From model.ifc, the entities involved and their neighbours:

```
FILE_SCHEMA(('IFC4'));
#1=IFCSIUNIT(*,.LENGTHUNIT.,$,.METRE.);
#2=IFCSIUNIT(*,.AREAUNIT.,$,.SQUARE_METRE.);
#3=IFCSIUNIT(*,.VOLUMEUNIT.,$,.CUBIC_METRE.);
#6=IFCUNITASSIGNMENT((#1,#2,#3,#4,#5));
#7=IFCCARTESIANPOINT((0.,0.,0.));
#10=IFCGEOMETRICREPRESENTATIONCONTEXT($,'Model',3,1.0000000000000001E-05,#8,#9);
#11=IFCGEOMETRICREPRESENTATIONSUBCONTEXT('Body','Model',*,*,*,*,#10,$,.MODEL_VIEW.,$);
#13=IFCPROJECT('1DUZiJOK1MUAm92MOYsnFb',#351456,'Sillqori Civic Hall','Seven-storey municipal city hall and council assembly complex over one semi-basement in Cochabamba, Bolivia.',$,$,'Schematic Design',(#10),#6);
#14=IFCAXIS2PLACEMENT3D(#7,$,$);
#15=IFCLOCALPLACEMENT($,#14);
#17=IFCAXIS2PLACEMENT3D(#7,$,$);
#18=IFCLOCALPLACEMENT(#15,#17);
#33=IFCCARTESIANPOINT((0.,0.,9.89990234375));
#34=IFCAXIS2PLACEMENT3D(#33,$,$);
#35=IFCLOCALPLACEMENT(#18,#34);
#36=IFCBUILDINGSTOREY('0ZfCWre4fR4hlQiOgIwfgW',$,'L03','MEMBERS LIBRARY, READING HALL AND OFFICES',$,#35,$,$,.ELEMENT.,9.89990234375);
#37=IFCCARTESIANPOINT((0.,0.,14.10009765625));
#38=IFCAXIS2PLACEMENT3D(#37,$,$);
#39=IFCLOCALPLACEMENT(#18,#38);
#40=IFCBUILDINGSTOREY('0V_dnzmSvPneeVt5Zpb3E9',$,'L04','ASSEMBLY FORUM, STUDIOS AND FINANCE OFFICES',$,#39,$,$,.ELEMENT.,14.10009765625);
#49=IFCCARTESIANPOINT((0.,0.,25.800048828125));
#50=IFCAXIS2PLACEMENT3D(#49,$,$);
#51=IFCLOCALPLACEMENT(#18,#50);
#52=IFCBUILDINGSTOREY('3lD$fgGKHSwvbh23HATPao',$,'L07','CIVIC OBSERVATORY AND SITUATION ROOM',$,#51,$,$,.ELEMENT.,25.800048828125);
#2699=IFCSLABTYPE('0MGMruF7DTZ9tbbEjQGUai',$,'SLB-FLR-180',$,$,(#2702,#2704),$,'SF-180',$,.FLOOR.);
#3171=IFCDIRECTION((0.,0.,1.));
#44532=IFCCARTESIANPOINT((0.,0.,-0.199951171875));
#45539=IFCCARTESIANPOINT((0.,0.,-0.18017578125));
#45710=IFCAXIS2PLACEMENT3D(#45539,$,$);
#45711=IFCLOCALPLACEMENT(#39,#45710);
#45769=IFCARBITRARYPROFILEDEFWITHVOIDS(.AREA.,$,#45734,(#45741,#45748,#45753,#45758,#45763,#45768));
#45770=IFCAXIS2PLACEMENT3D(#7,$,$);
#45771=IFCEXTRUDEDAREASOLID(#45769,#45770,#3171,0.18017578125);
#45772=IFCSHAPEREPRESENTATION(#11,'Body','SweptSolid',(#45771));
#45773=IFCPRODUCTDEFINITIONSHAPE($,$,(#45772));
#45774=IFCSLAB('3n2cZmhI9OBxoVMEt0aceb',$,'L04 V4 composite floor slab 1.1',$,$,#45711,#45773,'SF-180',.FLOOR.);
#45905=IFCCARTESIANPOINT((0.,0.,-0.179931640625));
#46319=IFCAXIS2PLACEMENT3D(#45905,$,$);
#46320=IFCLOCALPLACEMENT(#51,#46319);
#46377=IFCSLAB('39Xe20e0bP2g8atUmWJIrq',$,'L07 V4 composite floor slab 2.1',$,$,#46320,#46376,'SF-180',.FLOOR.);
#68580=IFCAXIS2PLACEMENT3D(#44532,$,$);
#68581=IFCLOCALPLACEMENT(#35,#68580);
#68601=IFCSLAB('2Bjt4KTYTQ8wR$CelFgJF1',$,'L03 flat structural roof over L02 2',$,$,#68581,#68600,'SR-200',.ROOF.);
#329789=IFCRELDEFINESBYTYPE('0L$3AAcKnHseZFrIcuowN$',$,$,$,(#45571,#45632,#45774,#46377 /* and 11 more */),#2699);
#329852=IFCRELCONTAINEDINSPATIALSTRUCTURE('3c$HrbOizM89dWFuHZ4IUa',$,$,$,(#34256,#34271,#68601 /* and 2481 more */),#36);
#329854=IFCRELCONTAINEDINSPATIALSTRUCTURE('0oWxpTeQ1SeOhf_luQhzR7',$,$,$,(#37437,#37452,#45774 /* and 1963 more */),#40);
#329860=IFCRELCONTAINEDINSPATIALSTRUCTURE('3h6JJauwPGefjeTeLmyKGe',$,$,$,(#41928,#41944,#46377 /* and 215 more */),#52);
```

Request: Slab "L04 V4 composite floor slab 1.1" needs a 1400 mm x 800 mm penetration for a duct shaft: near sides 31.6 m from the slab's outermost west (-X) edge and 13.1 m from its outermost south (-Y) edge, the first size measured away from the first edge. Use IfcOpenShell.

```python
import numpy as np
import ifcopenshell
import ifcopenshell.api.feature
import ifcopenshell.api.geometry
import ifcopenshell.api.root
import ifcopenshell.geom
import ifcopenshell.util.placement
import ifcopenshell.util.representation
import ifcopenshell.util.shape
import ifcopenshell.util.unit

model = ifcopenshell.open("model.ifc")
unit_scale = ifcopenshell.util.unit.calculate_unit_scale(model)
settings = ifcopenshell.geom.settings()


def volume(element):
    """Net volume in cubic metres, openings subtracted."""
    shape = ifcopenshell.geom.create_shape(settings, element)
    return ifcopenshell.util.shape.get_volume(shape.geometry)


slab = model.by_guid("3n2cZmhI9OBxoVMEt0aceb")
before = volume(slab)

# Extent in the slab's own axes, in metres. The edges named are its -X and -Y sides.
slab_shape = ifcopenshell.geom.create_shape(settings, slab)
vertices = ifcopenshell.util.shape.get_vertices(slab_shape.geometry)
x_min, y_min, bottom = vertices.min(axis=0)
top = vertices[:, 2].max()

opening = ifcopenshell.api.root.create_entity(model, ifc_class="IfcOpeningElement", name="Duct shaft opening", predefined_type="OPENING")
context = ifcopenshell.util.representation.get_context(model, "Model", "Body", "MODEL_VIEW")
width, depth = 1.4, 0.8
outline = [(0.0, 0.0), (width, 0.0), (width, depth), (0.0, depth), (0.0, 0.0)]
# Overshoot both faces by 50 mm so the cut is clean.
shape = ifcopenshell.api.geometry.add_slab_representation(
    model, context=context, depth=top - bottom + 0.1, polyline=outline
)
ifcopenshell.api.geometry.assign_representation(model, product=opening, representation=shape)

matrix = ifcopenshell.util.placement.get_local_placement(slab.ObjectPlacement)
matrix[:, 3] = matrix @ np.append(np.array([x_min + 31.6, y_min + 13.1, bottom - 0.05]) / unit_scale, 1.0)
ifcopenshell.api.geometry.edit_object_placement(model, product=opening, matrix=matrix, is_si=False)
ifcopenshell.api.feature.add_feature(model, feature=opening, element=slab)

after = volume(slab)

print(f"slab volume {before:.3f} -> {after:.3f} m3")

model.write("model_v2.ifc")
```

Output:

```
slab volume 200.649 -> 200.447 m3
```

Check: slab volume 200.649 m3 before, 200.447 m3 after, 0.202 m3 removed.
